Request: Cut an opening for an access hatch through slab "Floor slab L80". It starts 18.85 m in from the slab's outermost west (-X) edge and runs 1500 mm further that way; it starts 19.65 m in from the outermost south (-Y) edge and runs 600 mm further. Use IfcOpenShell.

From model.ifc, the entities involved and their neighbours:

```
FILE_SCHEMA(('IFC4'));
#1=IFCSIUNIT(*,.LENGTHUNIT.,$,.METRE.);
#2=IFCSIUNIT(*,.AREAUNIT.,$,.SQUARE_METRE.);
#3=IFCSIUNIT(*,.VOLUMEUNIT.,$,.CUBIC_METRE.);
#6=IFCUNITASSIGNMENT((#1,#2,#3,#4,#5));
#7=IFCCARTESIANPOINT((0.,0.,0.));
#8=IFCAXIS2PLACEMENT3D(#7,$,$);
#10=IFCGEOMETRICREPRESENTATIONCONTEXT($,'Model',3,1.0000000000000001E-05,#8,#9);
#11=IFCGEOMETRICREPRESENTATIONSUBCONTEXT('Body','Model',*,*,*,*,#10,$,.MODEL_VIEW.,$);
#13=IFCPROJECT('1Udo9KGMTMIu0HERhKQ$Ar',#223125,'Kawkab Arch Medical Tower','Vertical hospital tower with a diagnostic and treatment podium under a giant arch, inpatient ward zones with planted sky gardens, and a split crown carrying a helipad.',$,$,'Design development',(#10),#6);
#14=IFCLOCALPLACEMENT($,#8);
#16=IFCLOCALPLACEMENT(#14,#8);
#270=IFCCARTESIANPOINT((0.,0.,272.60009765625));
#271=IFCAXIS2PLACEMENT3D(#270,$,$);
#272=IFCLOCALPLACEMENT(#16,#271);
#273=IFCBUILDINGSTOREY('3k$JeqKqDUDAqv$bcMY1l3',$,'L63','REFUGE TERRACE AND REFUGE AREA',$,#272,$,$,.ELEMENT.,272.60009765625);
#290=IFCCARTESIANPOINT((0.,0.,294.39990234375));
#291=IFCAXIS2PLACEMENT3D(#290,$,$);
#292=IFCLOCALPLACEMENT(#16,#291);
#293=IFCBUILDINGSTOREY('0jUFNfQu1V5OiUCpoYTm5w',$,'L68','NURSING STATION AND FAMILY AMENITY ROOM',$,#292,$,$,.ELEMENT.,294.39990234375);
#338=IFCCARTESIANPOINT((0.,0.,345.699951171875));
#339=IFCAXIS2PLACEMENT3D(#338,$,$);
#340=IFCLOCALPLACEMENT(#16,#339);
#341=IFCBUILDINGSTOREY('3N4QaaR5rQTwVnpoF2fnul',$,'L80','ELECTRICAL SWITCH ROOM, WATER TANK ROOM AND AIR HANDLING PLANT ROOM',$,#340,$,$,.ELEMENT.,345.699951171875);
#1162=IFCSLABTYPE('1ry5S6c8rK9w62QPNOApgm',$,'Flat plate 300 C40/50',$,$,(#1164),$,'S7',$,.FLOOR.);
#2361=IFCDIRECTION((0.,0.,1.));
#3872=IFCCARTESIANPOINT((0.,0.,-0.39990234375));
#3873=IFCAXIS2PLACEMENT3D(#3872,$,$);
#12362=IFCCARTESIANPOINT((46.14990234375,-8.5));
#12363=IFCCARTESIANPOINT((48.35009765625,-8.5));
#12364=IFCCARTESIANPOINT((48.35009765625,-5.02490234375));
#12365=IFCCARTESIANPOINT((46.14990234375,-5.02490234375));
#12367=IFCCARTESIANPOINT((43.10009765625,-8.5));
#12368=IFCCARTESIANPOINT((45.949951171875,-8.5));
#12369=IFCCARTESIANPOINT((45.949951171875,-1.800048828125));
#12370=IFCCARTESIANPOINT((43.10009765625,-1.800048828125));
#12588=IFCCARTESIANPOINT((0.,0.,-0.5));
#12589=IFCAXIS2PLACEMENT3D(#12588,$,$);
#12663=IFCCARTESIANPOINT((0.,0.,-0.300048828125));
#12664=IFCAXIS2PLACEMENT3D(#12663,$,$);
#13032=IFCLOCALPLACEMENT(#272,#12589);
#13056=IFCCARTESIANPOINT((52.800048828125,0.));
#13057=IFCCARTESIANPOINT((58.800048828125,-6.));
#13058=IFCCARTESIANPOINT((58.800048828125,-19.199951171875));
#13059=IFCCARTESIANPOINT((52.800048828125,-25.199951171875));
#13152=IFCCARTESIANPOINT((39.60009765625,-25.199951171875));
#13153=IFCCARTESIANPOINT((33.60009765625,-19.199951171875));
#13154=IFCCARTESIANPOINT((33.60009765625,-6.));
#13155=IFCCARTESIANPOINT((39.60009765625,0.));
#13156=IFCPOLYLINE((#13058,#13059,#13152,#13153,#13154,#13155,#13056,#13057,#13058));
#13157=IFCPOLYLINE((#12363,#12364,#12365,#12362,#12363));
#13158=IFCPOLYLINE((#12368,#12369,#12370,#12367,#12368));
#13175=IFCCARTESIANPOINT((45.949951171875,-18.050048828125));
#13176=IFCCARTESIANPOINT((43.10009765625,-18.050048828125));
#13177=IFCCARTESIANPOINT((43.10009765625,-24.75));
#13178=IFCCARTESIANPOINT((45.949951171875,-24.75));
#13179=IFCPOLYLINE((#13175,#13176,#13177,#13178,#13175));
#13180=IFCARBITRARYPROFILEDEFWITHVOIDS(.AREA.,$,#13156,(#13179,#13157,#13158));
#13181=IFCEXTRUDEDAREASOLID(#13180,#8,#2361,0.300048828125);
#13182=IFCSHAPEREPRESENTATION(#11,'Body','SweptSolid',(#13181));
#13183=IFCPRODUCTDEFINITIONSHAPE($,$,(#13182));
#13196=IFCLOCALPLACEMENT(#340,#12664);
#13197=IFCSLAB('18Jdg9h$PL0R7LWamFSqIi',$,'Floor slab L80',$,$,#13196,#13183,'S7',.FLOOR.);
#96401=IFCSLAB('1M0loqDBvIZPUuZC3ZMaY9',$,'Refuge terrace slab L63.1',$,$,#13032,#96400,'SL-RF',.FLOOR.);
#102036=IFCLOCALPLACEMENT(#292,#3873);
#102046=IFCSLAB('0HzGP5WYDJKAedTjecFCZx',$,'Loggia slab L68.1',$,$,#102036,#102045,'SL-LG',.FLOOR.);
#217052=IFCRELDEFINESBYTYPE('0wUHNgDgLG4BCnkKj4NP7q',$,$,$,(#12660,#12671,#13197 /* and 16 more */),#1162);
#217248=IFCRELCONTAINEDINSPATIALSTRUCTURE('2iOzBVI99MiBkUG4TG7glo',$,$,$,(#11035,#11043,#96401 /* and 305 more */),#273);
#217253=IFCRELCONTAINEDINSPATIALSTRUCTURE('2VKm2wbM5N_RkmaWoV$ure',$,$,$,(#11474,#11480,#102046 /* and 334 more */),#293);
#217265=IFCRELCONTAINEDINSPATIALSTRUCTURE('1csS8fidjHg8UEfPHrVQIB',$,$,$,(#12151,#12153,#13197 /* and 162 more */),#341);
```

```python
import numpy as np
import ifcopenshell
import ifcopenshell.api.feature
import ifcopenshell.api.geometry
import ifcopenshell.api.root
import ifcopenshell.geom
import ifcopenshell.util.placement
import ifcopenshell.util.representation
import ifcopenshell.util.shape
import ifcopenshell.util.unit

model = ifcopenshell.open("model.ifc")
unit_scale = ifcopenshell.util.unit.calculate_unit_scale(model)
settings = ifcopenshell.geom.settings()


def volume(element):
    """Net volume in cubic metres, openings subtracted."""
    shape = ifcopenshell.geom.create_shape(settings, element)
    return ifcopenshell.util.shape.get_volume(shape.geometry)


slab = model.by_guid("18Jdg9h$PL0R7LWamFSqIi")
before = volume(slab)

# Extent in the slab's own axes, in metres. The edges named are its -X and -Y sides.
slab_shape = ifcopenshell.geom.create_shape(settings, slab)
vertices = ifcopenshell.util.shape.get_vertices(slab_shape.geometry)
x_min, y_min, bottom = vertices.min(axis=0)
top = vertices[:, 2].max()

opening = ifcopenshell.api.root.create_entity(model, ifc_class="IfcOpeningElement", name="Access hatch opening", predefined_type="OPENING")
context = ifcopenshell.util.representation.get_context(model, "Model", "Body", "MODEL_VIEW")
width, depth = 1.5, 0.6
outline = [(0.0, 0.0), (width, 0.0), (width, depth), (0.0, depth), (0.0, 0.0)]
# Overshoot both faces by 50 mm so the cut is clean.
shape = ifcopenshell.api.geometry.add_slab_representation(
    model, context=context, depth=top - bottom + 0.1, polyline=outline
)
ifcopenshell.api.geometry.assign_representation(model, product=opening, representation=shape)

matrix = ifcopenshell.util.placement.get_local_placement(slab.ObjectPlacement)
matrix[:, 3] = matrix @ np.append(np.array([x_min + 18.85, y_min + 19.65, bottom - 0.05]) / unit_scale, 1.0)
ifcopenshell.api.geometry.edit_object_placement(model, product=opening, matrix=matrix, is_si=False)
ifcopenshell.api.feature.add_feature(model, feature=opening, element=slab)

after = volume(slab)

print(f"slab volume {before:.3f} -> {after:.3f} m3")

model.write("model-out.ifc")
```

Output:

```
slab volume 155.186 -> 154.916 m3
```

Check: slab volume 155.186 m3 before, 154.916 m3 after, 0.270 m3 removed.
